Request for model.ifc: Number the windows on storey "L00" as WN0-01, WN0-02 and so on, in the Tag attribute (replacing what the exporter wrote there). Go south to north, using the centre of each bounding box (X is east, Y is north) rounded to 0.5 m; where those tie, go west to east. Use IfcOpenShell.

First a look at what the model holds.

```python
import ifcopenshell
import ifcopenshell.util.element
import ifcopenshell.util.placement

model = ifcopenshell.open("model.ifc")
print(model.schema)
storey = next(s for s in model.by_type("IfcBuildingStorey") if s.Name == "L00")
windows = [e for e in ifcopenshell.util.element.get_decomposition(storey) if e.is_a("IfcWindow")]
for e in sorted(windows, key=lambda e: e.id()):
    origin = ifcopenshell.util.placement.get_local_placement(e.ObjectPlacement)[:3, 3]
    print(e.id(), e.Tag, e.Name, origin.round(2) + 0.0, sep=" | ")
```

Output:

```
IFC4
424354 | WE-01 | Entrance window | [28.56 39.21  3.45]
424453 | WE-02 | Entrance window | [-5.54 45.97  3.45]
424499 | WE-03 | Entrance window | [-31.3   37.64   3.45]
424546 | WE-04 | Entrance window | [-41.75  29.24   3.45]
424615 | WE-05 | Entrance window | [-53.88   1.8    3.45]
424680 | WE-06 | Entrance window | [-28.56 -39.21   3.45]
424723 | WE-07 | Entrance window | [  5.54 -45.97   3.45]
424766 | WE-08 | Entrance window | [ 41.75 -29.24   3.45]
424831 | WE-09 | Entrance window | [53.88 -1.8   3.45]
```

```python
import ifcopenshell
import ifcopenshell.geom
import ifcopenshell.util.element
import ifcopenshell.util.shape

model = ifcopenshell.open("model.ifc")
settings = ifcopenshell.geom.settings()
settings.set("use-world-coords", True)


def centre(element):
    shape = ifcopenshell.geom.create_shape(settings, element)
    return ifcopenshell.util.shape.get_bbox_centroid(shape.geometry)


storey = next(s for s in model.by_type("IfcBuildingStorey") if s.Name == "L00")
windows = [e for e in ifcopenshell.util.element.get_decomposition(storey) if e.is_a("IfcWindow")]

# Insertion points can sit at a corner or the storey origin, so sort by the geometry (in metres).
centres = {e: centre(e) for e in windows}
windows.sort(key=lambda e: (round(centres[e][1] / 0.5), centres[e][0]))

for i, e in enumerate(windows, start=1):
    number = f"WN0-{i:02d}"
    e.Tag = number
    print(e.id(), number)

model.write("model_v2.ifc")
```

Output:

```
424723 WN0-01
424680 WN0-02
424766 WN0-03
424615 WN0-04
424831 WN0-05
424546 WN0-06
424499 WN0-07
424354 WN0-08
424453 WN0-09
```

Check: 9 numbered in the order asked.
